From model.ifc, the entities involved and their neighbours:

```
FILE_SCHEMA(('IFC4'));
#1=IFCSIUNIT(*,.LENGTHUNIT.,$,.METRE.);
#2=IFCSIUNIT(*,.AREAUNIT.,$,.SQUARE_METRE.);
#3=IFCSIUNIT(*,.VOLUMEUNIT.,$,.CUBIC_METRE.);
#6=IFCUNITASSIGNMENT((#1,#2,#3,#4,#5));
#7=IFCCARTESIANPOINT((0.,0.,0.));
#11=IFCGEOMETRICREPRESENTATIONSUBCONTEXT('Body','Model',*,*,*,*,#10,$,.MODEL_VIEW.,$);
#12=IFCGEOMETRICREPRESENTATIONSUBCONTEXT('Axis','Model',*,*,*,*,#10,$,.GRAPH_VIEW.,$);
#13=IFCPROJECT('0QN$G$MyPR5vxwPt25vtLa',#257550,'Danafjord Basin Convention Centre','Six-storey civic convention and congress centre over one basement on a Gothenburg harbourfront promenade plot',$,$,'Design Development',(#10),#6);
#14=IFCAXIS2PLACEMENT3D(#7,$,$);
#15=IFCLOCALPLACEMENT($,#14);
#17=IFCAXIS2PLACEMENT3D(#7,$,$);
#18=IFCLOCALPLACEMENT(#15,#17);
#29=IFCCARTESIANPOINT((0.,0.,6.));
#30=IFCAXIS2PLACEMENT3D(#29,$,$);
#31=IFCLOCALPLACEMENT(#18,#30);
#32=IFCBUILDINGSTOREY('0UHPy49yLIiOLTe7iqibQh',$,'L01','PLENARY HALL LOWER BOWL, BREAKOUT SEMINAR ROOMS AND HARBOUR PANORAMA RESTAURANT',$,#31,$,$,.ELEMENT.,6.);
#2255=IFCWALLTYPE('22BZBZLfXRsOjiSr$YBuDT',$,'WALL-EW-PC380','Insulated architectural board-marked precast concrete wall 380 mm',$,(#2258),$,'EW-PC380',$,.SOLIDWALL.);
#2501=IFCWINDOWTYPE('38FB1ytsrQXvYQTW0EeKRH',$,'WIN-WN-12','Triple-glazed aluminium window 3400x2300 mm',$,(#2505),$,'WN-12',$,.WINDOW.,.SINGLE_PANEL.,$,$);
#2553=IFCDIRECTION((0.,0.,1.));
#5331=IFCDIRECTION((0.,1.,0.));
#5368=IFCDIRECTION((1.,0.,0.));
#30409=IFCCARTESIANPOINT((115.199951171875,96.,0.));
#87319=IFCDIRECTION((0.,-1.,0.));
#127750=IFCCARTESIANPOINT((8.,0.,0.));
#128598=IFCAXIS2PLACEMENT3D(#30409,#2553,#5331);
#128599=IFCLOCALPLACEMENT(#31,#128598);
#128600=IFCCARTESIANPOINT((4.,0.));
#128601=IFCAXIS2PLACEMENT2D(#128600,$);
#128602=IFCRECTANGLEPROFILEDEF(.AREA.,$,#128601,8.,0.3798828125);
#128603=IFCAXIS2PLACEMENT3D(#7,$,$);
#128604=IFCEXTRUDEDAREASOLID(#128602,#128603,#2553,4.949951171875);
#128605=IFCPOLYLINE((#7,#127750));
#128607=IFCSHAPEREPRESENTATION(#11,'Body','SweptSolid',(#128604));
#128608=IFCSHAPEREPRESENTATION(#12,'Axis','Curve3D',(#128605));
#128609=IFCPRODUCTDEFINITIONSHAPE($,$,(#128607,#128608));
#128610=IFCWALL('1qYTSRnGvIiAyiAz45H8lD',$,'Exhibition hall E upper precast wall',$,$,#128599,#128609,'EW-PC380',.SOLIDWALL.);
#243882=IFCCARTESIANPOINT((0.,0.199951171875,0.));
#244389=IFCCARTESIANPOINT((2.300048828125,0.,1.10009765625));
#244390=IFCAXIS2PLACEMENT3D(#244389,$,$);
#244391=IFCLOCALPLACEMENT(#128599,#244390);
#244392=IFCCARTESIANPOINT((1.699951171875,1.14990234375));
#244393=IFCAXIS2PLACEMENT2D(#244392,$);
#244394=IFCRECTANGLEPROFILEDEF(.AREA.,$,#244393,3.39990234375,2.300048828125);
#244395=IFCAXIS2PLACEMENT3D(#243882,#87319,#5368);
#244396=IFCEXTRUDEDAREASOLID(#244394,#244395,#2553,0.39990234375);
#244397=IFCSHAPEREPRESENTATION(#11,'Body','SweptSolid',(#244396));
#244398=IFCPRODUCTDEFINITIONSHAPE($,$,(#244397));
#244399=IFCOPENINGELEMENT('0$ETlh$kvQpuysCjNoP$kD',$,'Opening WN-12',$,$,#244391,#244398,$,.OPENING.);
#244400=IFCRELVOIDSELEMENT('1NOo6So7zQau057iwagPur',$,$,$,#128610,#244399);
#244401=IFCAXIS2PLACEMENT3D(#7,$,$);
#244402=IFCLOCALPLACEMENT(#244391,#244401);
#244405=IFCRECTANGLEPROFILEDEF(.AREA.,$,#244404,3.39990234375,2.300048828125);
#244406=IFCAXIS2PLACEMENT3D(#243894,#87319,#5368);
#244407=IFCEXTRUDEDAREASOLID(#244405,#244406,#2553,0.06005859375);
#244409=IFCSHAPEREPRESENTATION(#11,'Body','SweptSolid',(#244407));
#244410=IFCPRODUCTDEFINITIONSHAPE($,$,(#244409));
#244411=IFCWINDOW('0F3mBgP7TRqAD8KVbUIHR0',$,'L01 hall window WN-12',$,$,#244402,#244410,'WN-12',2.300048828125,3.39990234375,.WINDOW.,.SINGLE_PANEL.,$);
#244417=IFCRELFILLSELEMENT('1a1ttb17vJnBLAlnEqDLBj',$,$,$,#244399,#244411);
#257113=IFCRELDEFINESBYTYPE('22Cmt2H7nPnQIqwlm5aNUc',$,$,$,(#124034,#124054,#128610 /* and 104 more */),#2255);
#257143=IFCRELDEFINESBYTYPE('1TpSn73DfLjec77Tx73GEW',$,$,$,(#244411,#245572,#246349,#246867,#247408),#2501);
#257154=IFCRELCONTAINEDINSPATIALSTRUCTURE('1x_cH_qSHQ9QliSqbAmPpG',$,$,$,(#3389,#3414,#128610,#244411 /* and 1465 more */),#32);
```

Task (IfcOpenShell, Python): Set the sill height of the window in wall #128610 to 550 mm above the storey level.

```python
import numpy as np
import ifcopenshell
import ifcopenshell.api.geometry
import ifcopenshell.geom
import ifcopenshell.util.element
import ifcopenshell.util.placement
import ifcopenshell.util.shape
import ifcopenshell.util.unit

model = ifcopenshell.open("model.ifc")
unit_scale = ifcopenshell.util.unit.calculate_unit_scale(model)

window = model.by_guid("0F3mBgP7TRqAD8KVbUIHR0")
opening = window.FillsVoids[0].RelatingOpeningElement
storey = ifcopenshell.util.element.get_container(window, ifc_class="IfcBuildingStorey")
level = ifcopenshell.util.placement.get_local_placement(storey.ObjectPlacement)[2, 3]

# The opening's origin need not be at the sill, so measure its lowest point.
shape = ifcopenshell.geom.create_shape(ifcopenshell.geom.settings(), opening)
bottom = ifcopenshell.util.shape.get_shape_bottom_elevation(shape, shape.geometry) / unit_scale
dz = level + 0.55 / unit_scale - bottom

shift = np.array([0.0, 0.0, dz])
# The window is placed relative to its opening, so it follows when the opening moves.
matrix = ifcopenshell.util.placement.get_local_placement(opening.ObjectPlacement)
matrix[:3, 3] += shift
ifcopenshell.api.geometry.edit_object_placement(
    model, product=opening, matrix=matrix, is_si=False, should_transform_children=True
)

print(f"moved by {dz * unit_scale:+.3f} m")

model.write("model_rev.ifc")
```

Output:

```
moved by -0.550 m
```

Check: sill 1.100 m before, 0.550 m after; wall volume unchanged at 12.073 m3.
